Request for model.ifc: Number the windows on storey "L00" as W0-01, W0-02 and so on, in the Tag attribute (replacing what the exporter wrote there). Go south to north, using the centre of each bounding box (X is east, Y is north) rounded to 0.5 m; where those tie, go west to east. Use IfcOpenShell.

First a look at what the model holds.

```python
import ifcopenshell
import ifcopenshell.util.element
import ifcopenshell.util.placement

model = ifcopenshell.open("model.ifc")
print(model.schema)
storey = next(s for s in model.by_type("IfcBuildingStorey") if s.Name == "L00")
windows = [e for e in ifcopenshell.util.element.get_decomposition(storey) if e.is_a("IfcWindow")]
for e in sorted(windows, key=lambda e: e.id()):
    origin = ifcopenshell.util.placement.get_local_placement(e.ObjectPlacement)[:3, 3]
    print(e.id(), e.Tag, e.Name, origin.round(2) + 0.0, sep=" | ")
```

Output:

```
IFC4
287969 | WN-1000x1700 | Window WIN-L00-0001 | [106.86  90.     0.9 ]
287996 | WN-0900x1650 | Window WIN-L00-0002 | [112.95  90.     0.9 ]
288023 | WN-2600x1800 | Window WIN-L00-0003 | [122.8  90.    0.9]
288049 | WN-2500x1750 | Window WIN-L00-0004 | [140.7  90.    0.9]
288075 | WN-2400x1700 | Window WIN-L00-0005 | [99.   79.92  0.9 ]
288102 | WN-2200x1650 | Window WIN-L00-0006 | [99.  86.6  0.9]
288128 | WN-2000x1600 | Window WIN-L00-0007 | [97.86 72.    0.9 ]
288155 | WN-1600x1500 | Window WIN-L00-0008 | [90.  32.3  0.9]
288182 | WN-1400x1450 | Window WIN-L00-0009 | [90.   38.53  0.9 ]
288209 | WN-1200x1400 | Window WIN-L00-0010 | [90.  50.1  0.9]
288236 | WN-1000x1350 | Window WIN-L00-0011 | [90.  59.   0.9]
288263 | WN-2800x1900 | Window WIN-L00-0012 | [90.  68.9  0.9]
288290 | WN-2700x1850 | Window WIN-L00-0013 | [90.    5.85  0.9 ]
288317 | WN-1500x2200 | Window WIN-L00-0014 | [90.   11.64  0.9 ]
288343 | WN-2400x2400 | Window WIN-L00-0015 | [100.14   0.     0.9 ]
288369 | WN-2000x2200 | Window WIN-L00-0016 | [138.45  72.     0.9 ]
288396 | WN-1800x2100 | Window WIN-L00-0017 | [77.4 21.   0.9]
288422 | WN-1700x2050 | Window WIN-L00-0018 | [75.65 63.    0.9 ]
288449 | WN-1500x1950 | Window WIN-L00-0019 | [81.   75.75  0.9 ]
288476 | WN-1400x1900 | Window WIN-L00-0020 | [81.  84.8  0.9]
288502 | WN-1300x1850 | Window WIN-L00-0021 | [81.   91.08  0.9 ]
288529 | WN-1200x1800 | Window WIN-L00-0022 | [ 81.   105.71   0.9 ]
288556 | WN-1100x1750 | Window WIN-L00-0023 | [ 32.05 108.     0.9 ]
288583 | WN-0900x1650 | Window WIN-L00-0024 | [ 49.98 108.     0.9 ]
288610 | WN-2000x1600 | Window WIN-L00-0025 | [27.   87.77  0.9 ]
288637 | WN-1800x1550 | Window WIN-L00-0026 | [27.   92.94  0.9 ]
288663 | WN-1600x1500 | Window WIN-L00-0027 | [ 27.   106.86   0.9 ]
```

```python
import ifcopenshell
import ifcopenshell.geom
import ifcopenshell.util.element
import ifcopenshell.util.shape

model = ifcopenshell.open("model.ifc")
settings = ifcopenshell.geom.settings()
settings.set("use-world-coords", True)


def centre(element):
    shape = ifcopenshell.geom.create_shape(settings, element)
    return ifcopenshell.util.shape.get_bbox_centroid(shape.geometry)


storey = next(s for s in model.by_type("IfcBuildingStorey") if s.Name == "L00")
windows = [e for e in ifcopenshell.util.element.get_decomposition(storey) if e.is_a("IfcWindow")]

# Insertion points can sit at a corner or the storey origin, so sort by the geometry (in metres).
centres = {e: centre(e) for e in windows}
windows.sort(key=lambda e: (round(centres[e][1] / 0.5), centres[e][0]))

for i, e in enumerate(windows, start=1):
    number = f"W0-{i:02d}"
    e.Tag = number
    print(e.id(), number)

model.write("model_rev.ifc")
```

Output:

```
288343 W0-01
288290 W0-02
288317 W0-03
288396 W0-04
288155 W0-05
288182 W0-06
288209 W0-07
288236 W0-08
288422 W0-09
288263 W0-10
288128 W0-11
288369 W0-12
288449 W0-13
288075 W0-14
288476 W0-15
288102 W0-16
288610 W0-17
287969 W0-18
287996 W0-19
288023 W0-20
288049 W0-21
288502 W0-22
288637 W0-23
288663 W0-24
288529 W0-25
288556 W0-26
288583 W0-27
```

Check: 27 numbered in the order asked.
